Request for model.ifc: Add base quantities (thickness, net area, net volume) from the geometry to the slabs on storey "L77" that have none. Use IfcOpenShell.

First a look at what the model holds.

```python
import ifcopenshell
import ifcopenshell.util.element
import ifcopenshell.util.unit

model = ifcopenshell.open("model.ifc")
print(model.schema)
for unit_type in ("LENGTHUNIT", "AREAUNIT", "VOLUMEUNIT"):
    print(unit_type, ifcopenshell.util.unit.calculate_unit_scale(model, unit_type))
storey = next(s for s in model.by_type("IfcBuildingStorey") if s.Name == "L77")
slabs = [e for e in ifcopenshell.util.element.get_decomposition(storey) if e.is_a("IfcSlab")]
for e in sorted(slabs, key=lambda e: e.id()):
    print(e.id(), e.is_a(), e.Name, list(ifcopenshell.util.element.get_psets(e, qtos_only=True)), sep=" | ")
```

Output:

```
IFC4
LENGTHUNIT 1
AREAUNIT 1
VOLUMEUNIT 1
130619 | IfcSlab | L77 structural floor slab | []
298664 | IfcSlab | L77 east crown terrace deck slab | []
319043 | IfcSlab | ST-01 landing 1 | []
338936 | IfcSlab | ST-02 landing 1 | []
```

```python
import ifcopenshell
import ifcopenshell.api.pset
import ifcopenshell.geom
import ifcopenshell.util.element
import ifcopenshell.util.shape
import ifcopenshell.util.unit

model = ifcopenshell.open("model.ifc")
unit_scale = ifcopenshell.util.unit.calculate_unit_scale(model)
area_scale = ifcopenshell.util.unit.calculate_unit_scale(model, "AREAUNIT")
volume_scale = ifcopenshell.util.unit.calculate_unit_scale(model, "VOLUMEUNIT")
settings = ifcopenshell.geom.settings()

storey = next(s for s in model.by_type("IfcBuildingStorey") if s.Name == "L77")
slabs = [e for e in ifcopenshell.util.element.get_decomposition(storey) if e.is_a("IfcSlab")]

for e in sorted(slabs, key=lambda e: e.id()):
    if ifcopenshell.util.element.get_psets(e, qtos_only=True, should_inherit=False):
        continue
    # Geometry comes back in metres, in the element's own axes.
    shape = ifcopenshell.geom.create_shape(settings, e)
    values = {
        "Width": ifcopenshell.util.shape.get_z(shape.geometry) / unit_scale,
        "NetArea": ifcopenshell.util.shape.get_footprint_area(shape.geometry) / area_scale,
        "NetVolume": ifcopenshell.util.shape.get_volume(shape.geometry) / volume_scale,
    }
    qto = ifcopenshell.api.pset.add_qto(model, product=e, name="Qto_SlabBaseQuantities")
    ifcopenshell.api.pset.edit_qto(model, qto=qto, properties=values)
    print(e.id(), {k: round(v, 3) for k, v in values.items()})

model.write("model_edited.ifc")
```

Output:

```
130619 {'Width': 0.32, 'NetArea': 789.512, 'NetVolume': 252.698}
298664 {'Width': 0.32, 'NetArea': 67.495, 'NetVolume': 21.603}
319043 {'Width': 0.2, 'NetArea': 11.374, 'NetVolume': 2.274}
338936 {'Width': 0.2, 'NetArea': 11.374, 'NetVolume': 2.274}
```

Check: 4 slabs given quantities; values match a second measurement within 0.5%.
